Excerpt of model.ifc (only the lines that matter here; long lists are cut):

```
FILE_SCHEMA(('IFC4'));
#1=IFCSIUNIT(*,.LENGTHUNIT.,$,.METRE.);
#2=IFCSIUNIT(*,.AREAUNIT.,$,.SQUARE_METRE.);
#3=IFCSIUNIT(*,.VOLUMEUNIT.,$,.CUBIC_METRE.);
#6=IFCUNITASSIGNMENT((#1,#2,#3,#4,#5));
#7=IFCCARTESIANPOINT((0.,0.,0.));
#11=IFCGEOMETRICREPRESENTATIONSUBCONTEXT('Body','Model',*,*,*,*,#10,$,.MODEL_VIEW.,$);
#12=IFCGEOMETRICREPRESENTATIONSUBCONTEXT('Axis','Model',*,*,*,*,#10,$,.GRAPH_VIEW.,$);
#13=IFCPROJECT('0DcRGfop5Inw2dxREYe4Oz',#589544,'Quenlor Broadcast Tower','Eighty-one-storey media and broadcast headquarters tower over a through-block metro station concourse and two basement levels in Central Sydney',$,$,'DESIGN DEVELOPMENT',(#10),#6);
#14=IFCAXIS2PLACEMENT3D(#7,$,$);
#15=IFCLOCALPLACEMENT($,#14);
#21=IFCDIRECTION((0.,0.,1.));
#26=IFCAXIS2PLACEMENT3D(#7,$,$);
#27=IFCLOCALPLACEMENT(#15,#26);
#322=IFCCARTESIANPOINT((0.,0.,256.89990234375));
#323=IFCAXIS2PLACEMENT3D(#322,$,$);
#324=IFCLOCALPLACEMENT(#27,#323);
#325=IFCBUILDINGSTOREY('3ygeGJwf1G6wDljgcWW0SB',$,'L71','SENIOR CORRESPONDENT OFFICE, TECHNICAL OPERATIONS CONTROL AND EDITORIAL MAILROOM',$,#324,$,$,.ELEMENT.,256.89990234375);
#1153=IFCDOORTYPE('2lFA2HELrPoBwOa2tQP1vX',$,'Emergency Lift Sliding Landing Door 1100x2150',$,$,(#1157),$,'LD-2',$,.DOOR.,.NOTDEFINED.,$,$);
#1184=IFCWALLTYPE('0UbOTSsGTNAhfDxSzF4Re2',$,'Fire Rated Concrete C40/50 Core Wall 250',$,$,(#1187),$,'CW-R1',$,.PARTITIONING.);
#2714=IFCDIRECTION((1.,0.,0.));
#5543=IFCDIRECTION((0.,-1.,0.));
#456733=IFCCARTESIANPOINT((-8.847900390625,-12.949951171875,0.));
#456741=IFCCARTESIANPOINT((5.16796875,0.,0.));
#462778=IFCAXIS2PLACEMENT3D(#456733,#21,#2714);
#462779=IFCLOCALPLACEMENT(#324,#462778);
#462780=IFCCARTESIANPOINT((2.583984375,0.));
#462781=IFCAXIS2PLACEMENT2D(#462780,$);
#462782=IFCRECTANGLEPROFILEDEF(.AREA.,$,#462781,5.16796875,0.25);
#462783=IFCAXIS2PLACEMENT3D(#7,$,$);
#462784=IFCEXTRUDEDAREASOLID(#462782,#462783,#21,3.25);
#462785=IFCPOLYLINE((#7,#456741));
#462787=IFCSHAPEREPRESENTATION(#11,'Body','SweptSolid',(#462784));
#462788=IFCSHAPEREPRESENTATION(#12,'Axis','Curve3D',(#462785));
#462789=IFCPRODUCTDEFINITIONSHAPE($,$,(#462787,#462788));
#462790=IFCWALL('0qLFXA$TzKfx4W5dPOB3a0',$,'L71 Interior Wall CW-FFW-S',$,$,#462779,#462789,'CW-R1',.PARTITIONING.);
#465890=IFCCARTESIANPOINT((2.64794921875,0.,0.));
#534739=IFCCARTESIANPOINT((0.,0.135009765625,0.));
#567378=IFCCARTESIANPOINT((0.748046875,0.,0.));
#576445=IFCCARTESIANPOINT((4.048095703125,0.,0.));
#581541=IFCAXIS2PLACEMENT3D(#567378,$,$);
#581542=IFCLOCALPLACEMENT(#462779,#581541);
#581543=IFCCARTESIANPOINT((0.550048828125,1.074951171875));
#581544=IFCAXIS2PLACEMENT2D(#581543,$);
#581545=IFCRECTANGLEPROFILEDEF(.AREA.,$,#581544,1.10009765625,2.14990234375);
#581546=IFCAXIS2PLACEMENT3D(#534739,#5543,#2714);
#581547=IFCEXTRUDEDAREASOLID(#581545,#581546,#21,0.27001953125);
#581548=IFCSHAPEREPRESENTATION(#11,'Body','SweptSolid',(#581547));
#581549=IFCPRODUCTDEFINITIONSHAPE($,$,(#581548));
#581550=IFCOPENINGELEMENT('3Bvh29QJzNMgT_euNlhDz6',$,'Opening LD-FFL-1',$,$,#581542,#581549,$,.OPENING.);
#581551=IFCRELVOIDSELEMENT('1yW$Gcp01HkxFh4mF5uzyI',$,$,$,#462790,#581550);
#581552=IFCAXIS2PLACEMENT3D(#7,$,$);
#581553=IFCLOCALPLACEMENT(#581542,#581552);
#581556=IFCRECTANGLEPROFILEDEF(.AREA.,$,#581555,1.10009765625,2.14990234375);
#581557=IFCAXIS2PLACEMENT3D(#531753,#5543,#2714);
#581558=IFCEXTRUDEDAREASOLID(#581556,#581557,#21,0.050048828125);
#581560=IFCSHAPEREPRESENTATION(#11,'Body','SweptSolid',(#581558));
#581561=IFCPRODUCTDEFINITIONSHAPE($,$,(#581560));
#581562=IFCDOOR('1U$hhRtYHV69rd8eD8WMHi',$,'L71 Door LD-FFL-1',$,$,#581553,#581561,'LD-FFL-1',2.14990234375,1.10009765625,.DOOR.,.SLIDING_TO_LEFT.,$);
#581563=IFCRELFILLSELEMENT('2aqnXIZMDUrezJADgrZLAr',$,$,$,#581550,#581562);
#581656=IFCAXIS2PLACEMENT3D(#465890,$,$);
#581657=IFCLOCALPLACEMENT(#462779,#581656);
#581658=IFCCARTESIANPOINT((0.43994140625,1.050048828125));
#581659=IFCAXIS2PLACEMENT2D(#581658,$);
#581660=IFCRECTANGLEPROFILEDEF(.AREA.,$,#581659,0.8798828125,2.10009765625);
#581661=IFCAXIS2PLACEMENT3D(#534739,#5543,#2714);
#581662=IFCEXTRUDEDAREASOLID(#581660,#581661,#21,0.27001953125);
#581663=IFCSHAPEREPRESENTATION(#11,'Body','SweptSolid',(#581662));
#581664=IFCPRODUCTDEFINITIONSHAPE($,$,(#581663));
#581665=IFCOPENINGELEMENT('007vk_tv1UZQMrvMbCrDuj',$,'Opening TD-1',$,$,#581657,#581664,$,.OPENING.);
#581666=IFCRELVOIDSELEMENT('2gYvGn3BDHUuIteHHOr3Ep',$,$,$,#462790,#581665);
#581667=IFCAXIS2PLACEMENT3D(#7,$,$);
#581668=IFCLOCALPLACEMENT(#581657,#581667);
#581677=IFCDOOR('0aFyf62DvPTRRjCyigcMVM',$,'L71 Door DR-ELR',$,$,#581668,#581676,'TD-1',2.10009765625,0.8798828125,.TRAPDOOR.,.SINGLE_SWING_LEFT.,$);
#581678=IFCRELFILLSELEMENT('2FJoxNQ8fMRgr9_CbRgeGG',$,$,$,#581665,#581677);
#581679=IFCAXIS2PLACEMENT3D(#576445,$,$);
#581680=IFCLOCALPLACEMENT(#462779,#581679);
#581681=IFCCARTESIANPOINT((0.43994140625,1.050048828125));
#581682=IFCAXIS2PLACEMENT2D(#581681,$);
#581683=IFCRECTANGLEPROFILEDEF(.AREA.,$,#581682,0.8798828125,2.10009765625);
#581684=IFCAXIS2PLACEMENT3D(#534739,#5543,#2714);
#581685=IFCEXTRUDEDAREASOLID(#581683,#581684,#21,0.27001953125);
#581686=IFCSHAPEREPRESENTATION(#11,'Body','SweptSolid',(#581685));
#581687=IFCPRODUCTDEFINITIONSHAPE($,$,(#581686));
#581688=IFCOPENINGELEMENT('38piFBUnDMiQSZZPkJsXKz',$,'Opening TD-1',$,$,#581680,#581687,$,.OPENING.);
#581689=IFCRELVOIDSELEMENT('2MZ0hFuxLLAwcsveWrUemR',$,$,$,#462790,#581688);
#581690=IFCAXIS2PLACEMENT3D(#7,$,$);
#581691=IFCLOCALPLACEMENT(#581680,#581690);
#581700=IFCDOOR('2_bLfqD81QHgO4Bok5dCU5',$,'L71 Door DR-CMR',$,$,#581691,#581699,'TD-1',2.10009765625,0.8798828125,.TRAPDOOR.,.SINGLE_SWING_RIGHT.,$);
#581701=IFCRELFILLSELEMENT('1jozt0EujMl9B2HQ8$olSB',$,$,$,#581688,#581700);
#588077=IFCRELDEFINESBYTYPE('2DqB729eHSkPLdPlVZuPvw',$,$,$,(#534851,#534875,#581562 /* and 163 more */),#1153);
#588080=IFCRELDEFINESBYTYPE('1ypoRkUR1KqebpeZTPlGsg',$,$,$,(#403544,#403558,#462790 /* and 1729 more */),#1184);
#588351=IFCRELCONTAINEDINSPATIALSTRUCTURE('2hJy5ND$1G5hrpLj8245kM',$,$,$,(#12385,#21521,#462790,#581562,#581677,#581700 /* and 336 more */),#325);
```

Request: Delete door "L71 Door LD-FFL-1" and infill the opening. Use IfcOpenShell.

```python
import ifcopenshell
import ifcopenshell.api.feature
import ifcopenshell.api.root
import ifcopenshell.geom
import ifcopenshell.util.shape

model = ifcopenshell.open("model.ifc")
settings = ifcopenshell.geom.settings()


def volume(element):
    """Net volume in cubic metres, openings subtracted."""
    shape = ifcopenshell.geom.create_shape(settings, element)
    return ifcopenshell.util.shape.get_volume(shape.geometry)


door = model.by_guid("1U$hhRtYHV69rd8eD8WMHi")
opening = door.FillsVoids[0].RelatingOpeningElement
wall = opening.VoidsElements[0].RelatingBuildingElement
before = volume(wall)

ifcopenshell.api.root.remove_product(model, product=door)
ifcopenshell.api.feature.remove_feature(model, feature=opening)

after = volume(wall)

print(f"wall volume {before:.3f} -> {after:.3f} m3")

model.write("model_updated.ifc")
```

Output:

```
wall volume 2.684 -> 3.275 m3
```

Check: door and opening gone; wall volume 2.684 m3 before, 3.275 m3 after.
